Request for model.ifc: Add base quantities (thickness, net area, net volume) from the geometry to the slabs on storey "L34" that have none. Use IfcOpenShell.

First a look at what the model holds.

```python
import ifcopenshell
import ifcopenshell.util.element
import ifcopenshell.util.unit

model = ifcopenshell.open("model.ifc")
print(model.schema)
for unit_type in ("LENGTHUNIT", "AREAUNIT", "VOLUMEUNIT"):
    print(unit_type, ifcopenshell.util.unit.calculate_unit_scale(model, unit_type))
storey = next(s for s in model.by_type("IfcBuildingStorey") if s.Name == "L34")
slabs = [e for e in ifcopenshell.util.element.get_decomposition(storey) if e.is_a("IfcSlab")]
for e in sorted(slabs, key=lambda e: e.id()):
    print(e.id(), e.is_a(), e.Name, list(ifcopenshell.util.element.get_psets(e, qtos_only=True)), sep=" | ")
```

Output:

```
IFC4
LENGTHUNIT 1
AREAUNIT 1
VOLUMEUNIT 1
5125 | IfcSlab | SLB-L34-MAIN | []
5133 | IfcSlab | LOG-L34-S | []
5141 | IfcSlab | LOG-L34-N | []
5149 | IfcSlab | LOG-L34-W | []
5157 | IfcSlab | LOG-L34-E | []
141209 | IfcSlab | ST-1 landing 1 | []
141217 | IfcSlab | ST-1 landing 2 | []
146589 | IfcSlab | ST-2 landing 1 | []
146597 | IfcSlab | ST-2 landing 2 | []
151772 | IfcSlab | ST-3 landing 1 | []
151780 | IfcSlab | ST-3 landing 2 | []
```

```python
import ifcopenshell
import ifcopenshell.api.pset
import ifcopenshell.geom
import ifcopenshell.util.element
import ifcopenshell.util.shape
import ifcopenshell.util.unit

model = ifcopenshell.open("model.ifc")
unit_scale = ifcopenshell.util.unit.calculate_unit_scale(model)
area_scale = ifcopenshell.util.unit.calculate_unit_scale(model, "AREAUNIT")
volume_scale = ifcopenshell.util.unit.calculate_unit_scale(model, "VOLUMEUNIT")
settings = ifcopenshell.geom.settings()

storey = next(s for s in model.by_type("IfcBuildingStorey") if s.Name == "L34")
slabs = [e for e in ifcopenshell.util.element.get_decomposition(storey) if e.is_a("IfcSlab")]

for e in sorted(slabs, key=lambda e: e.id()):
    if ifcopenshell.util.element.get_psets(e, qtos_only=True, should_inherit=False):
        continue
    # Geometry comes back in metres, in the element's own axes.
    shape = ifcopenshell.geom.create_shape(settings, e)
    values = {
        "Width": ifcopenshell.util.shape.get_z(shape.geometry) / unit_scale,
        "NetArea": ifcopenshell.util.shape.get_footprint_area(shape.geometry) / area_scale,
        "NetVolume": ifcopenshell.util.shape.get_volume(shape.geometry) / volume_scale,
    }
    qto = ifcopenshell.api.pset.add_qto(model, product=e, name="Qto_SlabBaseQuantities")
    ifcopenshell.api.pset.edit_qto(model, qto=qto, properties=values)
    print(e.id(), {k: round(v, 3) for k, v in values.items()})

model.write("model_edited.ifc")
```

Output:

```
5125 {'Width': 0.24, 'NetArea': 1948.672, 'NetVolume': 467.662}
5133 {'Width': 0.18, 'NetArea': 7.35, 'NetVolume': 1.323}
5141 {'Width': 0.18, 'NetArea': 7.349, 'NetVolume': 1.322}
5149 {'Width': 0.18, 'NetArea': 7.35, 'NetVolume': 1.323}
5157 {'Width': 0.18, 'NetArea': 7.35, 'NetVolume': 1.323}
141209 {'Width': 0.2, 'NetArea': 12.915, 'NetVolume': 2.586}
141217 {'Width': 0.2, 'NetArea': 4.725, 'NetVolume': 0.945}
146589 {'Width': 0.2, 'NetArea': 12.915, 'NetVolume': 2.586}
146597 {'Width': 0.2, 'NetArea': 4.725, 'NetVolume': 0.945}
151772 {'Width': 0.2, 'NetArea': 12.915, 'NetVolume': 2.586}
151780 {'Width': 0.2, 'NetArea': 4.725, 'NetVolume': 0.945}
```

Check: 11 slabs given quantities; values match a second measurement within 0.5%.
